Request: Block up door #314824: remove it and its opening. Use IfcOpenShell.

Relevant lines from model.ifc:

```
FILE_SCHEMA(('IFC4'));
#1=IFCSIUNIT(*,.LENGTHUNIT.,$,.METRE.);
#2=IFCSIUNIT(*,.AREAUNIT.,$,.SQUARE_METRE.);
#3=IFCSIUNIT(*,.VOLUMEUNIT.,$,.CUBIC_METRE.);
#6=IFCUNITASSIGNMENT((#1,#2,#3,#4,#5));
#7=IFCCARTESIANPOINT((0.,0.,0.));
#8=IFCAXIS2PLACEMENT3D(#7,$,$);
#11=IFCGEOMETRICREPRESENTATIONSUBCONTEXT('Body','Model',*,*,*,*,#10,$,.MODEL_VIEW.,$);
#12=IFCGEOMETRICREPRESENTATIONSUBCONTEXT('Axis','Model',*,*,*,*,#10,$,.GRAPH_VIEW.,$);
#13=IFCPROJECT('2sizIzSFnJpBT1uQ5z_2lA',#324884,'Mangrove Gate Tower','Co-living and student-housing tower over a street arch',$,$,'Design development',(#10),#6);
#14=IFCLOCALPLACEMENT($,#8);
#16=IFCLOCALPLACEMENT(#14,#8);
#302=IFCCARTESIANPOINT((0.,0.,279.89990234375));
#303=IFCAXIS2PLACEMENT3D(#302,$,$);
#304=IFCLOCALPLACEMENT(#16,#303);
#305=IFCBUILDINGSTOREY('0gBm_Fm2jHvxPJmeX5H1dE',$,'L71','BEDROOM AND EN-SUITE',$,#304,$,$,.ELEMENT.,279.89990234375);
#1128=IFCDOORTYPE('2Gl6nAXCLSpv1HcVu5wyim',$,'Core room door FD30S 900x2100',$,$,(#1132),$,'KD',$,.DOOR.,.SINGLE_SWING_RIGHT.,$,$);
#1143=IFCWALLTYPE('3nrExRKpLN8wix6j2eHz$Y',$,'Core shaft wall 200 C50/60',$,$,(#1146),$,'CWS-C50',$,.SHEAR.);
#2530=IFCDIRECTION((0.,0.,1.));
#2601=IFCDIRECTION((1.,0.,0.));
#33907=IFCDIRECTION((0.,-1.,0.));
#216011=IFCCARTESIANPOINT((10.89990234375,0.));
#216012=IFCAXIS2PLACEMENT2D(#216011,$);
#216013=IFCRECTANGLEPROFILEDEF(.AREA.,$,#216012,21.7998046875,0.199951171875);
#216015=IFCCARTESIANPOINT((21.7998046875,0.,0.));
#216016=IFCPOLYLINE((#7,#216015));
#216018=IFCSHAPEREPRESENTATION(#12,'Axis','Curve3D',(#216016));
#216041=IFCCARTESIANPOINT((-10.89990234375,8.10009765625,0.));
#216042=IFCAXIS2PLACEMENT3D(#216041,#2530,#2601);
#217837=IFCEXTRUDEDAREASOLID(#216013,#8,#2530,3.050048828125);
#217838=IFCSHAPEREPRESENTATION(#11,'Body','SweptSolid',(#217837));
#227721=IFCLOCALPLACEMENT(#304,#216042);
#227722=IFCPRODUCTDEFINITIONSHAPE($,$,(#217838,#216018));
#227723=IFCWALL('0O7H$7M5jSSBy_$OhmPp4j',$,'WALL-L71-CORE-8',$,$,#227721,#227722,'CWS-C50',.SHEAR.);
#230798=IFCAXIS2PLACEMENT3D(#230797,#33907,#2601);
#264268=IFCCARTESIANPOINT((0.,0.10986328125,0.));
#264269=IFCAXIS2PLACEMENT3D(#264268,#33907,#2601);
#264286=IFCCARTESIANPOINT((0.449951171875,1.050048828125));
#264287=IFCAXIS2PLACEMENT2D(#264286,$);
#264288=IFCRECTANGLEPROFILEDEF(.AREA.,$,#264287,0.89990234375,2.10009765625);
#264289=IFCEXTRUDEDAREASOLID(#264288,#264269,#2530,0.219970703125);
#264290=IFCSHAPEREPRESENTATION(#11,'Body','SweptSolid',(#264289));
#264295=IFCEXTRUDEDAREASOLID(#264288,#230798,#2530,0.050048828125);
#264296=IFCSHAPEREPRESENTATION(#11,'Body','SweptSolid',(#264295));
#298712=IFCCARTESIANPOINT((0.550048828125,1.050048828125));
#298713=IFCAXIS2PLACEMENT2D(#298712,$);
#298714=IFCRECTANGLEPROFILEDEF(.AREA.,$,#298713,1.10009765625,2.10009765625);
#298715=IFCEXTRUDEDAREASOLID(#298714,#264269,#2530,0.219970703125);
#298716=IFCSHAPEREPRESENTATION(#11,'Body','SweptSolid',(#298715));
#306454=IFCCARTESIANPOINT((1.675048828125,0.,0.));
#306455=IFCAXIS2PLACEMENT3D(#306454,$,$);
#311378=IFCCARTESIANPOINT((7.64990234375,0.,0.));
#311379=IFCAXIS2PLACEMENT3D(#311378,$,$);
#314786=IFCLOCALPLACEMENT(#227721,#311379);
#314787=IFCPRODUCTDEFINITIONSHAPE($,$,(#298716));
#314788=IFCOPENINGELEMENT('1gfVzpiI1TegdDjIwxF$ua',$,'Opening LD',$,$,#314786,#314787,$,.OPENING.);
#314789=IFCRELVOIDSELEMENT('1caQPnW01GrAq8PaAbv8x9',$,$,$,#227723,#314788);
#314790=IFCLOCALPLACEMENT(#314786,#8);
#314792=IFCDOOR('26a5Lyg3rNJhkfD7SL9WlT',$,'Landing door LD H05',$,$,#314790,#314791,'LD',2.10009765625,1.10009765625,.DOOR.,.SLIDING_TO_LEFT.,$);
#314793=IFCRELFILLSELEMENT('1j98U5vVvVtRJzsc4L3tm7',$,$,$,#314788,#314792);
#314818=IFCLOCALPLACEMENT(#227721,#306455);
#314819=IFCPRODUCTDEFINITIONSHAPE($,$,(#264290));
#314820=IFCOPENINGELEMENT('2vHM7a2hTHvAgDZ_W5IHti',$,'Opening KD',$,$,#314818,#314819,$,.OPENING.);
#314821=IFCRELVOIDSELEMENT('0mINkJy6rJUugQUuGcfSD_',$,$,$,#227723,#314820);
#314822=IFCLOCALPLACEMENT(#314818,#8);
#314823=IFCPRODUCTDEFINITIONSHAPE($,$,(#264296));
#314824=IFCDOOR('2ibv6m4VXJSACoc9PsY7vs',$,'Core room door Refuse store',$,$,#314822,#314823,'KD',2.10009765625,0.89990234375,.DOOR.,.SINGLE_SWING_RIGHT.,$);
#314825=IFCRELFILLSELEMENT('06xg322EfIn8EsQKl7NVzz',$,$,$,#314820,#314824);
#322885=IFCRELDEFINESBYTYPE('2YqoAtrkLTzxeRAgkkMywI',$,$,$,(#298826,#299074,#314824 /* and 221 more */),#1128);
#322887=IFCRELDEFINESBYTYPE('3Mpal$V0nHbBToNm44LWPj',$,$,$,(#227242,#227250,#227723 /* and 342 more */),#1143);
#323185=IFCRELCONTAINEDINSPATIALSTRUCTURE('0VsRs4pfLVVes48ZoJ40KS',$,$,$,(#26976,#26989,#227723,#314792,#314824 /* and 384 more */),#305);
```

```python
import ifcopenshell
import ifcopenshell.api.feature
import ifcopenshell.api.root
import ifcopenshell.geom
import ifcopenshell.util.shape

model = ifcopenshell.open("model.ifc")
settings = ifcopenshell.geom.settings()


def volume(element):
    """Net volume in cubic metres, openings subtracted."""
    shape = ifcopenshell.geom.create_shape(settings, element)
    return ifcopenshell.util.shape.get_volume(shape.geometry)


door = model.by_id(314824)
opening = door.FillsVoids[0].RelatingOpeningElement
wall = opening.VoidsElements[0].RelatingBuildingElement
before = volume(wall)

ifcopenshell.api.root.remove_product(model, product=door)
ifcopenshell.api.feature.remove_feature(model, feature=opening)

after = volume(wall)

print(f"wall volume {before:.3f} -> {after:.3f} m3")

model.write("model_updated.ifc")
```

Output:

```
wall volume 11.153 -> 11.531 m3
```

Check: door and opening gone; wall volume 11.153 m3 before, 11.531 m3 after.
